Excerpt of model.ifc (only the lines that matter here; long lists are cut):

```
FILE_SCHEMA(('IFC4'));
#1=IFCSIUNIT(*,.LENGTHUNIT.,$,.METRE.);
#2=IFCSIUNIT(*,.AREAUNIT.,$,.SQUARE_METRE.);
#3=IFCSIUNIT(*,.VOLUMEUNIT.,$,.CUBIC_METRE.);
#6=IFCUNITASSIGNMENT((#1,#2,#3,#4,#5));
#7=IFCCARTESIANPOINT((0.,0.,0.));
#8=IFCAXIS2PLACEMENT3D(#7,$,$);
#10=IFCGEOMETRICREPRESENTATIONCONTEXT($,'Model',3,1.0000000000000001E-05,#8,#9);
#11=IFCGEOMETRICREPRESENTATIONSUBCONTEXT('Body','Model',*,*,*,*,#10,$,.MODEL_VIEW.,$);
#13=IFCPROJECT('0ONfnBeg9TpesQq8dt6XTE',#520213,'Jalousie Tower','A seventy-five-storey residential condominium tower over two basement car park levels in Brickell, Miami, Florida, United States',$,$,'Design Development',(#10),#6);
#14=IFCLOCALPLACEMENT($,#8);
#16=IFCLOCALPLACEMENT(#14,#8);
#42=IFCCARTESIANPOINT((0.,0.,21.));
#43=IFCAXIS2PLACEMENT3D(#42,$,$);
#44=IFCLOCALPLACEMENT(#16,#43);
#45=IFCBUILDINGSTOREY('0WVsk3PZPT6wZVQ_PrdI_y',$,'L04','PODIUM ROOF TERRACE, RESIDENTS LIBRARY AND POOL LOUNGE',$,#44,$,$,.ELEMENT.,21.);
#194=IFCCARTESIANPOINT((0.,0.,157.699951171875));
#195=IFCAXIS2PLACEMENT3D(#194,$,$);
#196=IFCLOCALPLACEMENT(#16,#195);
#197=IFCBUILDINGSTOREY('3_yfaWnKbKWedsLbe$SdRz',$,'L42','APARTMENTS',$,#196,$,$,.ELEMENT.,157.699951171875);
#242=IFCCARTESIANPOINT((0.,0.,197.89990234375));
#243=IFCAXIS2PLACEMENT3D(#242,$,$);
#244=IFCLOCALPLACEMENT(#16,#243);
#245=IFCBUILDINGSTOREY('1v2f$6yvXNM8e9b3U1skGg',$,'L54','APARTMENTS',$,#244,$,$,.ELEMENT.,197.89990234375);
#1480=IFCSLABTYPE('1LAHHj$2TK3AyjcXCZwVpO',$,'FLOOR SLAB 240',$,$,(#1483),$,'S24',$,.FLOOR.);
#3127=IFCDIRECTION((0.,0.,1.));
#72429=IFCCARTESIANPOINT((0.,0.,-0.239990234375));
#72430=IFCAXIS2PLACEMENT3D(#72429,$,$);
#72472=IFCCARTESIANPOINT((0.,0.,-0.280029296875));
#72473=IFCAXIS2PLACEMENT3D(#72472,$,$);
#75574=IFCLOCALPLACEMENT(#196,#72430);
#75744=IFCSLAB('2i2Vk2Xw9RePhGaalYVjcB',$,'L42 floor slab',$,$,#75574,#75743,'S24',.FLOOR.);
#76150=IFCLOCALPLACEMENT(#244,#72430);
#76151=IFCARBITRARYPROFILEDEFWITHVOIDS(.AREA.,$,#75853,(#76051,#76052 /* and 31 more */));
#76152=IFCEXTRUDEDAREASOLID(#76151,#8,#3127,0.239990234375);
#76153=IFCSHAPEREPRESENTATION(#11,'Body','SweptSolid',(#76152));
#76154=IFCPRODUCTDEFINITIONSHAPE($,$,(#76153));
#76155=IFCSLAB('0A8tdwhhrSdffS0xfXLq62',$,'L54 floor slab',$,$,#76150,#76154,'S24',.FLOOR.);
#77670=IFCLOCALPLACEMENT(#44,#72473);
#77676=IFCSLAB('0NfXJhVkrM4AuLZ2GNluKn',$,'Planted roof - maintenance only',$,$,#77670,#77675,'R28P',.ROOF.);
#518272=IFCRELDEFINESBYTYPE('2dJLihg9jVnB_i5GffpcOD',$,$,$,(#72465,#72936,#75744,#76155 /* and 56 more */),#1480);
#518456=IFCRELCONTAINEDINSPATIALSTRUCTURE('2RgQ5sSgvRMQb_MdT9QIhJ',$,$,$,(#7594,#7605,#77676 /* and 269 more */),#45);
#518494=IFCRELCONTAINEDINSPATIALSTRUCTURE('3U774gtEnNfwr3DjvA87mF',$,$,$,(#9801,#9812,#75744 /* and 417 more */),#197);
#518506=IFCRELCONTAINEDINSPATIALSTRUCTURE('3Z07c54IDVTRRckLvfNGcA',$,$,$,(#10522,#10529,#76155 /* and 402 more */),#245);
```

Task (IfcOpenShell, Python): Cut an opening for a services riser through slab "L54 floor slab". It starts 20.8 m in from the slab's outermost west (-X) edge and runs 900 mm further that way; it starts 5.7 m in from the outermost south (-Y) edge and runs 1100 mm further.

```python
import numpy as np
import ifcopenshell
import ifcopenshell.api.feature
import ifcopenshell.api.geometry
import ifcopenshell.api.root
import ifcopenshell.geom
import ifcopenshell.util.placement
import ifcopenshell.util.representation
import ifcopenshell.util.shape
import ifcopenshell.util.unit

model = ifcopenshell.open("model.ifc")
unit_scale = ifcopenshell.util.unit.calculate_unit_scale(model)
settings = ifcopenshell.geom.settings()


def volume(element):
    """Net volume in cubic metres, openings subtracted."""
    shape = ifcopenshell.geom.create_shape(settings, element)
    return ifcopenshell.util.shape.get_volume(shape.geometry)


slab = model.by_id(76155)
before = volume(slab)

# Extent in the slab's own axes, in metres. The edges named are its -X and -Y sides.
slab_shape = ifcopenshell.geom.create_shape(settings, slab)
vertices = ifcopenshell.util.shape.get_vertices(slab_shape.geometry)
x_min, y_min, bottom = vertices.min(axis=0)
top = vertices[:, 2].max()

opening = ifcopenshell.api.root.create_entity(model, ifc_class="IfcOpeningElement", name="Services riser opening", predefined_type="OPENING")
context = ifcopenshell.util.representation.get_context(model, "Model", "Body", "MODEL_VIEW")
width, depth = 0.9, 1.1
outline = [(0.0, 0.0), (width, 0.0), (width, depth), (0.0, depth), (0.0, 0.0)]
# Overshoot both faces by 50 mm so the cut is clean.
shape = ifcopenshell.api.geometry.add_slab_representation(
    model, context=context, depth=top - bottom + 0.1, polyline=outline
)
ifcopenshell.api.geometry.assign_representation(model, product=opening, representation=shape)

matrix = ifcopenshell.util.placement.get_local_placement(slab.ObjectPlacement)
matrix[:, 3] = matrix @ np.append(np.array([x_min + 20.8, y_min + 5.7, bottom - 0.05]) / unit_scale, 1.0)
ifcopenshell.api.geometry.edit_object_placement(model, product=opening, matrix=matrix, is_si=False)
ifcopenshell.api.feature.add_feature(model, feature=opening, element=slab)

after = volume(slab)

print(f"slab volume {before:.3f} -> {after:.3f} m3")

model.write("model_rev.ifc")
```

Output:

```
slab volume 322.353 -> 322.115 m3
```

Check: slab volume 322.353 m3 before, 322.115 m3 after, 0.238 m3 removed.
